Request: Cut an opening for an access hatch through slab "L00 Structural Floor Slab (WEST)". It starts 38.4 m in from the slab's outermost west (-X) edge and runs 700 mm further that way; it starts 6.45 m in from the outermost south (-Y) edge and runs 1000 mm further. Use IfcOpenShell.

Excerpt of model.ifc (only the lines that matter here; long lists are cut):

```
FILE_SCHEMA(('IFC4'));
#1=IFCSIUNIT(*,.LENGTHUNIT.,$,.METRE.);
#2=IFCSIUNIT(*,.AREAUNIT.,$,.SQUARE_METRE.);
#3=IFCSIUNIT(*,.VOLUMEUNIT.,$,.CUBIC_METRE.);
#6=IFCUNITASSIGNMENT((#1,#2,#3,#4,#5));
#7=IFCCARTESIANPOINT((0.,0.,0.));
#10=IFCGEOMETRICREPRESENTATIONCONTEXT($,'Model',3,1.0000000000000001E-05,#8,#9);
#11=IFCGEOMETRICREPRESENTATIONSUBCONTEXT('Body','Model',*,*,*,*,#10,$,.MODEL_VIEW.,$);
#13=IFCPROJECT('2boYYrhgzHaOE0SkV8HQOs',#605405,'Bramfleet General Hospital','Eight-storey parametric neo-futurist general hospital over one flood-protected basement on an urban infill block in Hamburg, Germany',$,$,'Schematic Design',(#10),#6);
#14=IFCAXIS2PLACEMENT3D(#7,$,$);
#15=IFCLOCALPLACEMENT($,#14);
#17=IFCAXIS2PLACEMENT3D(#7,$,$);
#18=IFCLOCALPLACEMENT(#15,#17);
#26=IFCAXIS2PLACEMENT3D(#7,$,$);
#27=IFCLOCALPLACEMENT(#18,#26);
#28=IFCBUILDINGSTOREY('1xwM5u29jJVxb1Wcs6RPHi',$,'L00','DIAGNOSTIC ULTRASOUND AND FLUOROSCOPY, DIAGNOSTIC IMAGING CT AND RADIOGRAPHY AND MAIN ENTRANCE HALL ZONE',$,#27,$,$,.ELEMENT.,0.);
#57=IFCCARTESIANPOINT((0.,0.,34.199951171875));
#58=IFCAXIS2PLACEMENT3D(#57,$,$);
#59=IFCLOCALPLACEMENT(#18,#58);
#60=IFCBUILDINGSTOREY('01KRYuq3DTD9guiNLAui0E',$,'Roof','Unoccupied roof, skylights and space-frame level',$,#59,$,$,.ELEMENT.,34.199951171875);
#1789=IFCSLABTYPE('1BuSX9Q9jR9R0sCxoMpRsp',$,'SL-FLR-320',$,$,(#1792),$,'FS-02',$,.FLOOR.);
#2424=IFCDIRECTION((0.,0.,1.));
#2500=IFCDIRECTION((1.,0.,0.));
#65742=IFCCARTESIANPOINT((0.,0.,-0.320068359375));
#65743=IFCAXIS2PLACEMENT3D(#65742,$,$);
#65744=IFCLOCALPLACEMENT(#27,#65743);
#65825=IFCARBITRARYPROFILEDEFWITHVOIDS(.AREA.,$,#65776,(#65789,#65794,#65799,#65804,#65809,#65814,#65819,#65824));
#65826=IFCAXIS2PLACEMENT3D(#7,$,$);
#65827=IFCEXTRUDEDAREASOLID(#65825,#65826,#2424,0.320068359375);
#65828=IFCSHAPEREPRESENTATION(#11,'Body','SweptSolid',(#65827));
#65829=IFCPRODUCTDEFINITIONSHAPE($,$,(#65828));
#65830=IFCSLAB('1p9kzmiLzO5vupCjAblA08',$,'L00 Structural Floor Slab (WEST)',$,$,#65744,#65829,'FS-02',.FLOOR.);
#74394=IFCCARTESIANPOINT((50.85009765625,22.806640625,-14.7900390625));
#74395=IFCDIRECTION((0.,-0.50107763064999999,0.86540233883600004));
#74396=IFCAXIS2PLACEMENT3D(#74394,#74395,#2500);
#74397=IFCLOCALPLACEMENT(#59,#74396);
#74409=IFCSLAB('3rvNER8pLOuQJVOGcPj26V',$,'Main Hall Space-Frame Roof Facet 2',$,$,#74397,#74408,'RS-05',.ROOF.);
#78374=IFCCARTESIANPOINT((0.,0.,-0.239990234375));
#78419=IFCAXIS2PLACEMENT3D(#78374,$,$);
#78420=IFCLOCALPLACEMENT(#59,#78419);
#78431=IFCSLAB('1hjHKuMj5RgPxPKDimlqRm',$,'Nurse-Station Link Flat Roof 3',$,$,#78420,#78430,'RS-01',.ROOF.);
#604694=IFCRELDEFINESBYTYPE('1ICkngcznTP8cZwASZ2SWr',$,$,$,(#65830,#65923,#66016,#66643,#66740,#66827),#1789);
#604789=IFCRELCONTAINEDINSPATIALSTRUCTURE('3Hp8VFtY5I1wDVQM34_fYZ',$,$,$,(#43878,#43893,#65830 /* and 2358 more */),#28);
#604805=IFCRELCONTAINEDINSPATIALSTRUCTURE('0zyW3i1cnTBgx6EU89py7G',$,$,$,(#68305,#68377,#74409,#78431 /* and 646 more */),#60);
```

```python
import numpy as np
import ifcopenshell
import ifcopenshell.api.feature
import ifcopenshell.api.geometry
import ifcopenshell.api.root
import ifcopenshell.geom
import ifcopenshell.util.placement
import ifcopenshell.util.representation
import ifcopenshell.util.shape
import ifcopenshell.util.unit

model = ifcopenshell.open("model.ifc")
unit_scale = ifcopenshell.util.unit.calculate_unit_scale(model)
settings = ifcopenshell.geom.settings()


def volume(element):
    """Net volume in cubic metres, openings subtracted."""
    shape = ifcopenshell.geom.create_shape(settings, element)
    return ifcopenshell.util.shape.get_volume(shape.geometry)


slab = model.by_guid("1p9kzmiLzO5vupCjAblA08")
before = volume(slab)

# Extent in the slab's own axes, in metres. The edges named are its -X and -Y sides.
slab_shape = ifcopenshell.geom.create_shape(settings, slab)
vertices = ifcopenshell.util.shape.get_vertices(slab_shape.geometry)
x_min, y_min, bottom = vertices.min(axis=0)
top = vertices[:, 2].max()

opening = ifcopenshell.api.root.create_entity(model, ifc_class="IfcOpeningElement", name="Access hatch opening", predefined_type="OPENING")
context = ifcopenshell.util.representation.get_context(model, "Model", "Body", "MODEL_VIEW")
width, depth = 0.7, 1
outline = [(0.0, 0.0), (width, 0.0), (width, depth), (0.0, depth), (0.0, 0.0)]
# Overshoot both faces by 50 mm so the cut is clean.
shape = ifcopenshell.api.geometry.add_slab_representation(
    model, context=context, depth=top - bottom + 0.1, polyline=outline
)
ifcopenshell.api.geometry.assign_representation(model, product=opening, representation=shape)

matrix = ifcopenshell.util.placement.get_local_placement(slab.ObjectPlacement)
matrix[:, 3] = matrix @ np.append(np.array([x_min + 38.4, y_min + 6.45, bottom - 0.05]) / unit_scale, 1.0)
ifcopenshell.api.geometry.edit_object_placement(model, product=opening, matrix=matrix, is_si=False)
ifcopenshell.api.feature.add_feature(model, feature=opening, element=slab)

after = volume(slab)

print(f"slab volume {before:.3f} -> {after:.3f} m3")

model.write("model_v2.ifc")
```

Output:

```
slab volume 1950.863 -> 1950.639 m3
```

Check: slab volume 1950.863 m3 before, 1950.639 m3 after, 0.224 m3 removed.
